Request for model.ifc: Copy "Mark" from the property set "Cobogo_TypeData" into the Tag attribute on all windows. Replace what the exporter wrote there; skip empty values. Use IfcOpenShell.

First a look at what the model holds.

```python
import ifcopenshell
import ifcopenshell.util.element

model = ifcopenshell.open("model.ifc")
print(model.schema)
windows = model.by_type("IfcWindow")
print(len(windows), "windows")
for e in windows[:8]:
    source = ifcopenshell.util.element.get_pset(e, "Cobogo_TypeData", "Mark")
    target = e.Tag
    print(e.id(), repr(source), repr(target), sep=" | ")
```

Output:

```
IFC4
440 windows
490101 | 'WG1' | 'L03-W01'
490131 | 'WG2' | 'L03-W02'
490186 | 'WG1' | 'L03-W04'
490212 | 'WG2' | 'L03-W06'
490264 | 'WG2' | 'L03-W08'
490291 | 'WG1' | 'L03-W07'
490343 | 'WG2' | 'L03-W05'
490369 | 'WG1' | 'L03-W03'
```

```python
import ifcopenshell
import ifcopenshell.util.element

model = ifcopenshell.open("model.ifc")

count = 0
for e in model.by_type("IfcWindow"):
    value = ifcopenshell.util.element.get_pset(e, "Cobogo_TypeData", "Mark")
    current = e.Tag
    if not value or not value.strip() or current == value:
        continue
    e.Tag = value
    count += 1

print(count, "windows updated")

model.write("model_edited.ifc")
```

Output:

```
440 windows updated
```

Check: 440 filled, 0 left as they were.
